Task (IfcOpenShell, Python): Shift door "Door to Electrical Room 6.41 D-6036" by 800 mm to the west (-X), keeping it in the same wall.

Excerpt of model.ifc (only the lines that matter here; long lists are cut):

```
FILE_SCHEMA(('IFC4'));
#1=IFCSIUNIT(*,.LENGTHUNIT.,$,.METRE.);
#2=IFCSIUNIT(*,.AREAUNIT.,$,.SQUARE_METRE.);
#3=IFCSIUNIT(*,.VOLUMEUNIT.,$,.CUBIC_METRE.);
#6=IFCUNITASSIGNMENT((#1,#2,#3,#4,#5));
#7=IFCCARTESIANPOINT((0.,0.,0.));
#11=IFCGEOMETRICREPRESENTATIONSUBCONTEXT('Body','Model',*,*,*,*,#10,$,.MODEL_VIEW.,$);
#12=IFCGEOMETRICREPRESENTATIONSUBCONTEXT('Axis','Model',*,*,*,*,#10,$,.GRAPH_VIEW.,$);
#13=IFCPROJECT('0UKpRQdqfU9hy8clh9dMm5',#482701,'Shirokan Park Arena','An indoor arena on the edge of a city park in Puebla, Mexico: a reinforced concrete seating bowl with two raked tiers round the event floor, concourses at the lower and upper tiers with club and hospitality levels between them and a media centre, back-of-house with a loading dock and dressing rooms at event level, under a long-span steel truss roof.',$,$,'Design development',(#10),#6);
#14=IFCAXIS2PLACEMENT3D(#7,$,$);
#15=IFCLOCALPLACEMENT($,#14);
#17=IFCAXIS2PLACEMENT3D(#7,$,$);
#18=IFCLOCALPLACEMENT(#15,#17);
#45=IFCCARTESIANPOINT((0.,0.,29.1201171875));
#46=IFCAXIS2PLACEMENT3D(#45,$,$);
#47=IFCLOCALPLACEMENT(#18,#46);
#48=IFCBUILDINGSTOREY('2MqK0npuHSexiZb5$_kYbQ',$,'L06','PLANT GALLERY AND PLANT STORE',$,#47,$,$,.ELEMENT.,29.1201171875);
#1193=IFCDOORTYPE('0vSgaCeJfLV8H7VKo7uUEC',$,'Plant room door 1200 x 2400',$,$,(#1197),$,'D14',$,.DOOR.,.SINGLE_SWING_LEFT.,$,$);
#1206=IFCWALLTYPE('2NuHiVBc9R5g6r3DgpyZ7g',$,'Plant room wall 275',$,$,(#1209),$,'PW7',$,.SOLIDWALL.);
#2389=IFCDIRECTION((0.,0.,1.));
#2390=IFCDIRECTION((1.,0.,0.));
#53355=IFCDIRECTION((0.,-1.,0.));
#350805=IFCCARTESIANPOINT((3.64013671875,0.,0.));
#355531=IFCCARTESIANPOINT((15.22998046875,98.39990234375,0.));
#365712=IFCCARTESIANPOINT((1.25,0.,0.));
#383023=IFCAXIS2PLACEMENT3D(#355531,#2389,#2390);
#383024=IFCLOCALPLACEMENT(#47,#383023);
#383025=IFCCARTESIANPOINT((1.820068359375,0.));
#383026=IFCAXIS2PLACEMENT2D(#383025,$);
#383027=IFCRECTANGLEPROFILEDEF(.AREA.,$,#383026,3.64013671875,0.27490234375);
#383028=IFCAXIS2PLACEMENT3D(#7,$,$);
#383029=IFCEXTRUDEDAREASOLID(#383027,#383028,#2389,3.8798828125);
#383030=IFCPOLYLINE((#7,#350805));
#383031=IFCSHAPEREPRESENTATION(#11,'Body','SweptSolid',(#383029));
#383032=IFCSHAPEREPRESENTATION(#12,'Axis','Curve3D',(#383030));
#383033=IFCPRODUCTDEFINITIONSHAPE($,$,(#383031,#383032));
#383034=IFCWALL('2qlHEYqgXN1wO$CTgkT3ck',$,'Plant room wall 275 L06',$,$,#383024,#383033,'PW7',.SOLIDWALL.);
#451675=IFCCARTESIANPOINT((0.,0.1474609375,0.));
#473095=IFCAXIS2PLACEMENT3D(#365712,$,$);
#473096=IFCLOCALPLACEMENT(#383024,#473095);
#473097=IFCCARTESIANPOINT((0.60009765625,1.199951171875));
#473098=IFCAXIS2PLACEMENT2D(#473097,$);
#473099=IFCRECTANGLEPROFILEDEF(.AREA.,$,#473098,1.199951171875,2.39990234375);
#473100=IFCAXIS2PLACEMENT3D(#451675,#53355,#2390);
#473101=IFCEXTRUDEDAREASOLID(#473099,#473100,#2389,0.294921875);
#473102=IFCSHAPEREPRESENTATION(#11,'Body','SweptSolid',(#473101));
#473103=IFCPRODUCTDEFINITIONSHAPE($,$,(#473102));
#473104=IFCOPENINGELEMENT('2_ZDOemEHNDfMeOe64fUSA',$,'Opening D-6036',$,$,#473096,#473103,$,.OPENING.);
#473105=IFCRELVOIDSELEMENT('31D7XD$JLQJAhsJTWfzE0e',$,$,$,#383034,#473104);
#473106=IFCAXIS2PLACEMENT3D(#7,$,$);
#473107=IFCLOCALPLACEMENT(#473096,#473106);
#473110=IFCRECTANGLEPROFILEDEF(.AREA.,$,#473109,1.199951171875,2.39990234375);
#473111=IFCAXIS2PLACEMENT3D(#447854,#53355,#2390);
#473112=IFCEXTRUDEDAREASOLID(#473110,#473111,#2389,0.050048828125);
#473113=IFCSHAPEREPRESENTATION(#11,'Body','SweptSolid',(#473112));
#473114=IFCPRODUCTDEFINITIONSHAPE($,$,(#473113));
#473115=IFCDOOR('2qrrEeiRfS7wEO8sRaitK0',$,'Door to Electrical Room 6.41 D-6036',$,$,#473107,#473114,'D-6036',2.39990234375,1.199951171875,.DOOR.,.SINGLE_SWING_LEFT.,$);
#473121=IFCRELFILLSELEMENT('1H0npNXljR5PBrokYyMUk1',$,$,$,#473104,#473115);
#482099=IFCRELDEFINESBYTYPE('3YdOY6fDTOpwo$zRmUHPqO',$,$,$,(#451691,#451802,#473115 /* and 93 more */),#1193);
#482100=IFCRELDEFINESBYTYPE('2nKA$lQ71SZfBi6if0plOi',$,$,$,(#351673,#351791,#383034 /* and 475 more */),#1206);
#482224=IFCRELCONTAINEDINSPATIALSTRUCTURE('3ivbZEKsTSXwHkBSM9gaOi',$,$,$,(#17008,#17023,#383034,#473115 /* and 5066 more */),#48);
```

```python
import ifcopenshell
import ifcopenshell.api.geometry
import ifcopenshell.util.placement

model = ifcopenshell.open("model.ifc")

door = model.by_guid("2qrrEeiRfS7wEO8sRaitK0")
opening = door.FillsVoids[0].RelatingOpeningElement
wall = opening.VoidsElements[0].RelatingBuildingElement

wall_matrix = ifcopenshell.util.placement.get_local_placement(wall.ObjectPlacement)
shift = wall_matrix[:3, 0] * -0.8
before = ifcopenshell.util.placement.get_local_placement(door.ObjectPlacement)[:3, 3].copy()

# The door is placed relative to its opening, so it follows when the opening moves.
matrix = ifcopenshell.util.placement.get_local_placement(opening.ObjectPlacement)
matrix[:3, 3] += shift
ifcopenshell.api.geometry.edit_object_placement(
    model, product=opening, matrix=matrix, is_si=False, should_transform_children=True
)

after = ifcopenshell.util.placement.get_local_placement(door.ObjectPlacement)[:3, 3]
print("door moved by", (after - before).round(3) + 0.0)

model.write("model-out.ifc")
```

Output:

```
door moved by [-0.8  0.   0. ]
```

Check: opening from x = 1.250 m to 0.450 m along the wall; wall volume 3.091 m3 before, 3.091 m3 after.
